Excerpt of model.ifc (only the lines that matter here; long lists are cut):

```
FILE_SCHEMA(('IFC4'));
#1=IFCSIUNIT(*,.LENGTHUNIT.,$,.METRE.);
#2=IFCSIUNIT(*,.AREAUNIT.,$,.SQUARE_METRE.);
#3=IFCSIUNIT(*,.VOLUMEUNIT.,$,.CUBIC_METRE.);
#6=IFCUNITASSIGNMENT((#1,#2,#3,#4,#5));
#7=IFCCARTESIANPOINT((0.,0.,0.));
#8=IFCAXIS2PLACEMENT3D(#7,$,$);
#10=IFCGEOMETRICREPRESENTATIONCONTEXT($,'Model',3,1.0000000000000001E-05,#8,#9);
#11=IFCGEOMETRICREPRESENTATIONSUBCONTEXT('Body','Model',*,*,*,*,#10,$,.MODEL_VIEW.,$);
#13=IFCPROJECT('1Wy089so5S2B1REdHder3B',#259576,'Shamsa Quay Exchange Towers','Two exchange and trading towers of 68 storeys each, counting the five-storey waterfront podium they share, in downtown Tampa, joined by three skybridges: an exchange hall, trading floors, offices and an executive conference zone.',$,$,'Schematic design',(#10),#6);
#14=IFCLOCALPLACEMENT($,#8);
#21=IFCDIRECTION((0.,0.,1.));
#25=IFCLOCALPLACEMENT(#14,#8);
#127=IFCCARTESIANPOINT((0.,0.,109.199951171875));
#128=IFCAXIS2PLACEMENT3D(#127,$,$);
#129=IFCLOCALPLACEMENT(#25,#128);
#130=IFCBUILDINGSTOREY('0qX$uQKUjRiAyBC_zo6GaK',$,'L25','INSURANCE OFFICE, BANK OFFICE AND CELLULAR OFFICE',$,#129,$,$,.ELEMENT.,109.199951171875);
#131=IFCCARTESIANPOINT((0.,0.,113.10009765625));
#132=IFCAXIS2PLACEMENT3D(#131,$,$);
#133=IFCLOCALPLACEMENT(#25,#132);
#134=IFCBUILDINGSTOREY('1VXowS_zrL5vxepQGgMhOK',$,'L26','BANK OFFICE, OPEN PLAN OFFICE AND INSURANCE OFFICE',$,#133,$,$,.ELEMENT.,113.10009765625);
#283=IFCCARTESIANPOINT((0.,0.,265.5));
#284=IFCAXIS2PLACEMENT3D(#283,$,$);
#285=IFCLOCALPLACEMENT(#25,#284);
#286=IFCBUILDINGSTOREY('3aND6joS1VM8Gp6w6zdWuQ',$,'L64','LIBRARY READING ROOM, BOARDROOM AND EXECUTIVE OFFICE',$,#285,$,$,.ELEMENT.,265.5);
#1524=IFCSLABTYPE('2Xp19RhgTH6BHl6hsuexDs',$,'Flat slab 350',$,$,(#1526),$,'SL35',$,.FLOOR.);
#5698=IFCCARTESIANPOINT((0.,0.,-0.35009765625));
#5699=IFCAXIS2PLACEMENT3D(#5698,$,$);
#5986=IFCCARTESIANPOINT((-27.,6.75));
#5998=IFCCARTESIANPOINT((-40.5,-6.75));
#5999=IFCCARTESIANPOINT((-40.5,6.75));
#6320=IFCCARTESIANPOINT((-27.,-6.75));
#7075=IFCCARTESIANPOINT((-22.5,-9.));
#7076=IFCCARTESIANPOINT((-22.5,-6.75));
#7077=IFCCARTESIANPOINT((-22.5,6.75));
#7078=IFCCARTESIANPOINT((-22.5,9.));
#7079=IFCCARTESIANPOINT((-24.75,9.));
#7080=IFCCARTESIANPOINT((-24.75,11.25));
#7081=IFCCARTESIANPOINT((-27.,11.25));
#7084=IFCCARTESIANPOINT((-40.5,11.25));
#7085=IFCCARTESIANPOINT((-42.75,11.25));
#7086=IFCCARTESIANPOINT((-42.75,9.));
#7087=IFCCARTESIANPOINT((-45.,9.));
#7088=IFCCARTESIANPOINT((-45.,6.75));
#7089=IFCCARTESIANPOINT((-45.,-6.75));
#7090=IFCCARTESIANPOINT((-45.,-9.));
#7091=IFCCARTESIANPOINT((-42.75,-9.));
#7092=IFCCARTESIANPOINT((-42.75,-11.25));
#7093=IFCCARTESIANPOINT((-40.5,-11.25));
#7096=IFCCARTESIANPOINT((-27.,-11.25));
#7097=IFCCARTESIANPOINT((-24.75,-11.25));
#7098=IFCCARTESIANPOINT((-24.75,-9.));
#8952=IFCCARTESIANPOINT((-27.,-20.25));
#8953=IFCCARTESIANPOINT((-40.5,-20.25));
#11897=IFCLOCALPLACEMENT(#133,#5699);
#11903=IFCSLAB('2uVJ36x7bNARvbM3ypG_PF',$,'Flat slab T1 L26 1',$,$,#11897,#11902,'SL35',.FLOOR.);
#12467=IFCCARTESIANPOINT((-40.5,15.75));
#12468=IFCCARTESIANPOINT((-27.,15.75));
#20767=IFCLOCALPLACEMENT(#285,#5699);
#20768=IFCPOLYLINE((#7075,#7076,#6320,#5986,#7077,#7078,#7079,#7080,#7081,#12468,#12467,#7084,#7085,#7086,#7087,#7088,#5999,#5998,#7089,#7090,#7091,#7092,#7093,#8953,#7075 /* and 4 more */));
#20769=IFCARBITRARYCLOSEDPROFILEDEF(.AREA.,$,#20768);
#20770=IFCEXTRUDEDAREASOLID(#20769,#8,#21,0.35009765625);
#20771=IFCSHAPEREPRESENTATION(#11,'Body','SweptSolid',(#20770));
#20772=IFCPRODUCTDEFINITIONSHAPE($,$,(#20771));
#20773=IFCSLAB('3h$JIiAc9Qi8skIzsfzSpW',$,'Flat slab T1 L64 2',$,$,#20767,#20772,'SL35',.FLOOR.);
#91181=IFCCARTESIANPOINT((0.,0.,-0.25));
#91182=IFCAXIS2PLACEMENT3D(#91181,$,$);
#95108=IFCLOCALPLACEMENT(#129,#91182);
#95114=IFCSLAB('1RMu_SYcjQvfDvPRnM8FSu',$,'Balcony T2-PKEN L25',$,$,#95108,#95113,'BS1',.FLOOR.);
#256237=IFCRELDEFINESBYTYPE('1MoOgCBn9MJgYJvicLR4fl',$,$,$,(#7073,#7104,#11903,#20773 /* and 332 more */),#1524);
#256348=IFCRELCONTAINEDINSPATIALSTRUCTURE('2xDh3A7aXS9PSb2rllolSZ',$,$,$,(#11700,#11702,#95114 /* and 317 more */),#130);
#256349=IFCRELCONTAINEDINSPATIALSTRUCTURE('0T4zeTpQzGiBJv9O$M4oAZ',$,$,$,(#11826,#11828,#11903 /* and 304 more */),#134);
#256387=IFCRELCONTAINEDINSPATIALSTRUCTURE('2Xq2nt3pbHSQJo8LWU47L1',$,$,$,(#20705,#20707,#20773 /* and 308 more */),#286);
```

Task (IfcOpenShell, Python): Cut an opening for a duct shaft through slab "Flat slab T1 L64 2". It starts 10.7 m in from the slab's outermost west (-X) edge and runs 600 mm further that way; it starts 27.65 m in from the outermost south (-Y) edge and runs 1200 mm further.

```python
import numpy as np
import ifcopenshell
import ifcopenshell.api.feature
import ifcopenshell.api.geometry
import ifcopenshell.api.root
import ifcopenshell.geom
import ifcopenshell.util.placement
import ifcopenshell.util.representation
import ifcopenshell.util.shape
import ifcopenshell.util.unit

model = ifcopenshell.open("model.ifc")
unit_scale = ifcopenshell.util.unit.calculate_unit_scale(model)
settings = ifcopenshell.geom.settings()


def volume(element):
    """Net volume in cubic metres, openings subtracted."""
    shape = ifcopenshell.geom.create_shape(settings, element)
    return ifcopenshell.util.shape.get_volume(shape.geometry)


slab = model.by_guid("3h$JIiAc9Qi8skIzsfzSpW")
before = volume(slab)

# Extent in the slab's own axes, in metres. The edges named are its -X and -Y sides.
slab_shape = ifcopenshell.geom.create_shape(settings, slab)
vertices = ifcopenshell.util.shape.get_vertices(slab_shape.geometry)
x_min, y_min, bottom = vertices.min(axis=0)
top = vertices[:, 2].max()

opening = ifcopenshell.api.root.create_entity(model, ifc_class="IfcOpeningElement", name="Duct shaft opening", predefined_type="OPENING")
context = ifcopenshell.util.representation.get_context(model, "Model", "Body", "MODEL_VIEW")
width, depth = 0.6, 1.2
outline = [(0.0, 0.0), (width, 0.0), (width, depth), (0.0, depth), (0.0, 0.0)]
# Overshoot both faces by 50 mm so the cut is clean.
shape = ifcopenshell.api.geometry.add_slab_representation(
    model, context=context, depth=top - bottom + 0.1, polyline=outline
)
ifcopenshell.api.geometry.assign_representation(model, product=opening, representation=shape)

matrix = ifcopenshell.util.placement.get_local_placement(slab.ObjectPlacement)
matrix[:, 3] = matrix @ np.append(np.array([x_min + 10.7, y_min + 27.65, bottom - 0.05]) / unit_scale, 1.0)
ifcopenshell.api.geometry.edit_object_placement(model, product=opening, matrix=matrix, is_si=False)
ifcopenshell.api.feature.add_feature(model, feature=opening, element=slab)

after = volume(slab)

print(f"slab volume {before:.3f} -> {after:.3f} m3")

model.write("model_rev.ifc")
```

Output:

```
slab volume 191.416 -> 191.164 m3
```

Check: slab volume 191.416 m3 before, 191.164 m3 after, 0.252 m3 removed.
